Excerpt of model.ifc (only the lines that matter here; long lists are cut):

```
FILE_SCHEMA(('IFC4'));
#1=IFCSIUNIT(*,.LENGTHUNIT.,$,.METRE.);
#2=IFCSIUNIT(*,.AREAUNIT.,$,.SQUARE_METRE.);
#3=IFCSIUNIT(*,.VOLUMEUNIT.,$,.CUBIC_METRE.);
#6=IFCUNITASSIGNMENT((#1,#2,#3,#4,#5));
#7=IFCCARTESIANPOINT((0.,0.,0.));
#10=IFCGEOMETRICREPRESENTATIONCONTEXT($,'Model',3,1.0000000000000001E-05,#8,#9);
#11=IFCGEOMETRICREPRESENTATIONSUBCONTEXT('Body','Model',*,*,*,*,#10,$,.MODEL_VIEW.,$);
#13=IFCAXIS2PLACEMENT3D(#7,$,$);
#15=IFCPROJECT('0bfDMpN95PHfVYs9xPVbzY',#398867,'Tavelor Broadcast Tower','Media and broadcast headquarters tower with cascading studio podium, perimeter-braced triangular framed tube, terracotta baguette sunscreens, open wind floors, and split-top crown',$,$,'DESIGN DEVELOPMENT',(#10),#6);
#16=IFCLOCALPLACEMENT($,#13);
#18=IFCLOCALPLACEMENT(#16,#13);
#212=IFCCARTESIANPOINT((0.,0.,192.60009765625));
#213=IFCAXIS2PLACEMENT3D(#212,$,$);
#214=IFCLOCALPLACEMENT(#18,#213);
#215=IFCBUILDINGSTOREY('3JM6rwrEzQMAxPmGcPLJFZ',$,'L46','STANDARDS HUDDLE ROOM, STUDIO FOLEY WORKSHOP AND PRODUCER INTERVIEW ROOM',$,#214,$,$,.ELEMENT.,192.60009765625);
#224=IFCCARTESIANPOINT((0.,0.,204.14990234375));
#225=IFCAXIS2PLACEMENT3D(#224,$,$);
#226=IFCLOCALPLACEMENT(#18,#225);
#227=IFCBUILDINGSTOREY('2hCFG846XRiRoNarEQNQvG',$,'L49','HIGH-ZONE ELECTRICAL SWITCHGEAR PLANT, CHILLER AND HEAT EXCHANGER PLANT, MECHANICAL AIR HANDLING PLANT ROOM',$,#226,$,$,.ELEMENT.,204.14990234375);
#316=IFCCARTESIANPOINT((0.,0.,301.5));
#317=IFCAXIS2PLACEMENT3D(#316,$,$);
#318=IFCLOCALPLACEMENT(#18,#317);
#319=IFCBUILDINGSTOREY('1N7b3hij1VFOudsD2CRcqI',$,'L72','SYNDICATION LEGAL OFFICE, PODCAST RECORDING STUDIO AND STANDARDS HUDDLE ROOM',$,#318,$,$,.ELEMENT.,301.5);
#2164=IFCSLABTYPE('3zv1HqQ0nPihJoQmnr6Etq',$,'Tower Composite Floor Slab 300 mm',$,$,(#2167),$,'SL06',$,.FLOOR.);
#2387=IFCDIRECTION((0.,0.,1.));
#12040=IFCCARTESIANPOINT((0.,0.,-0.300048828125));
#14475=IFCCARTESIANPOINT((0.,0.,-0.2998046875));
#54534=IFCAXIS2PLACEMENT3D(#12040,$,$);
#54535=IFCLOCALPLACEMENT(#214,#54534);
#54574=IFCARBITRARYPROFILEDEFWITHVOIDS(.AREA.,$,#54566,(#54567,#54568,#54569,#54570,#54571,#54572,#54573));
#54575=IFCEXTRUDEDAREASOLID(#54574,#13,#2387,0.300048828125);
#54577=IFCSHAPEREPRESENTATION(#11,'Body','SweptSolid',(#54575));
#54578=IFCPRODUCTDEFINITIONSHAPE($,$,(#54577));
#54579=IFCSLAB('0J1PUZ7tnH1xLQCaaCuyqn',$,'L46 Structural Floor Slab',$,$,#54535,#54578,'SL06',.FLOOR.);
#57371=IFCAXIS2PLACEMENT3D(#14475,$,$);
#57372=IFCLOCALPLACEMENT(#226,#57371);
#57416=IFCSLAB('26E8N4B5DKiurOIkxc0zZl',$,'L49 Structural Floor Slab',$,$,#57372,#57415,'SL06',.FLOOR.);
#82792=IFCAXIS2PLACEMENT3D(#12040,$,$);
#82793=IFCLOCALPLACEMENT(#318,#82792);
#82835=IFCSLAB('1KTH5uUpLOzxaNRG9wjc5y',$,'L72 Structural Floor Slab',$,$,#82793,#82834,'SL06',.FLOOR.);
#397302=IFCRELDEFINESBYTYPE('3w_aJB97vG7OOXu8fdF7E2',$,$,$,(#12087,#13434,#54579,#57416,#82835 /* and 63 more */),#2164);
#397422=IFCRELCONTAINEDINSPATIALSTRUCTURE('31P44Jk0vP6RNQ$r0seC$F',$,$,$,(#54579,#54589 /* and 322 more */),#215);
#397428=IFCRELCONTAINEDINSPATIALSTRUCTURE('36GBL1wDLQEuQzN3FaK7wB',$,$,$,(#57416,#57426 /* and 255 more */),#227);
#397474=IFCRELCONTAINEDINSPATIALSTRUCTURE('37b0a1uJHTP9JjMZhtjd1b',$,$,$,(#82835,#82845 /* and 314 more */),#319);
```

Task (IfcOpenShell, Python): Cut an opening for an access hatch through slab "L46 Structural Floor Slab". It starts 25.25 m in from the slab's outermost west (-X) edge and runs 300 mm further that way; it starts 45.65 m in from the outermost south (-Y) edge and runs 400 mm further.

```python
import numpy as np
import ifcopenshell
import ifcopenshell.api.feature
import ifcopenshell.api.geometry
import ifcopenshell.api.root
import ifcopenshell.geom
import ifcopenshell.util.placement
import ifcopenshell.util.representation
import ifcopenshell.util.shape
import ifcopenshell.util.unit

model = ifcopenshell.open("model.ifc")
unit_scale = ifcopenshell.util.unit.calculate_unit_scale(model)
settings = ifcopenshell.geom.settings()


def volume(element):
    """Net volume in cubic metres, openings subtracted."""
    shape = ifcopenshell.geom.create_shape(settings, element)
    return ifcopenshell.util.shape.get_volume(shape.geometry)


slab = model.by_guid("0J1PUZ7tnH1xLQCaaCuyqn")
before = volume(slab)

# Extent in the slab's own axes, in metres. The edges named are its -X and -Y sides.
slab_shape = ifcopenshell.geom.create_shape(settings, slab)
vertices = ifcopenshell.util.shape.get_vertices(slab_shape.geometry)
x_min, y_min, bottom = vertices.min(axis=0)
top = vertices[:, 2].max()

opening = ifcopenshell.api.root.create_entity(model, ifc_class="IfcOpeningElement", name="Access hatch opening", predefined_type="OPENING")
context = ifcopenshell.util.representation.get_context(model, "Model", "Body", "MODEL_VIEW")
width, depth = 0.3, 0.4
outline = [(0.0, 0.0), (width, 0.0), (width, depth), (0.0, depth), (0.0, 0.0)]
# Overshoot both faces by 50 mm so the cut is clean.
shape = ifcopenshell.api.geometry.add_slab_representation(
    model, context=context, depth=top - bottom + 0.1, polyline=outline
)
ifcopenshell.api.geometry.assign_representation(model, product=opening, representation=shape)

matrix = ifcopenshell.util.placement.get_local_placement(slab.ObjectPlacement)
matrix[:, 3] = matrix @ np.append(np.array([x_min + 25.25, y_min + 45.65, bottom - 0.05]) / unit_scale, 1.0)
ifcopenshell.api.geometry.edit_object_placement(model, product=opening, matrix=matrix, is_si=False)
ifcopenshell.api.feature.add_feature(model, feature=opening, element=slab)

after = volume(slab)

print(f"slab volume {before:.3f} -> {after:.3f} m3")

model.write("model_updated.ifc")
```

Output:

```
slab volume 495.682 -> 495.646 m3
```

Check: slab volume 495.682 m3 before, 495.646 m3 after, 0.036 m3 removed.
